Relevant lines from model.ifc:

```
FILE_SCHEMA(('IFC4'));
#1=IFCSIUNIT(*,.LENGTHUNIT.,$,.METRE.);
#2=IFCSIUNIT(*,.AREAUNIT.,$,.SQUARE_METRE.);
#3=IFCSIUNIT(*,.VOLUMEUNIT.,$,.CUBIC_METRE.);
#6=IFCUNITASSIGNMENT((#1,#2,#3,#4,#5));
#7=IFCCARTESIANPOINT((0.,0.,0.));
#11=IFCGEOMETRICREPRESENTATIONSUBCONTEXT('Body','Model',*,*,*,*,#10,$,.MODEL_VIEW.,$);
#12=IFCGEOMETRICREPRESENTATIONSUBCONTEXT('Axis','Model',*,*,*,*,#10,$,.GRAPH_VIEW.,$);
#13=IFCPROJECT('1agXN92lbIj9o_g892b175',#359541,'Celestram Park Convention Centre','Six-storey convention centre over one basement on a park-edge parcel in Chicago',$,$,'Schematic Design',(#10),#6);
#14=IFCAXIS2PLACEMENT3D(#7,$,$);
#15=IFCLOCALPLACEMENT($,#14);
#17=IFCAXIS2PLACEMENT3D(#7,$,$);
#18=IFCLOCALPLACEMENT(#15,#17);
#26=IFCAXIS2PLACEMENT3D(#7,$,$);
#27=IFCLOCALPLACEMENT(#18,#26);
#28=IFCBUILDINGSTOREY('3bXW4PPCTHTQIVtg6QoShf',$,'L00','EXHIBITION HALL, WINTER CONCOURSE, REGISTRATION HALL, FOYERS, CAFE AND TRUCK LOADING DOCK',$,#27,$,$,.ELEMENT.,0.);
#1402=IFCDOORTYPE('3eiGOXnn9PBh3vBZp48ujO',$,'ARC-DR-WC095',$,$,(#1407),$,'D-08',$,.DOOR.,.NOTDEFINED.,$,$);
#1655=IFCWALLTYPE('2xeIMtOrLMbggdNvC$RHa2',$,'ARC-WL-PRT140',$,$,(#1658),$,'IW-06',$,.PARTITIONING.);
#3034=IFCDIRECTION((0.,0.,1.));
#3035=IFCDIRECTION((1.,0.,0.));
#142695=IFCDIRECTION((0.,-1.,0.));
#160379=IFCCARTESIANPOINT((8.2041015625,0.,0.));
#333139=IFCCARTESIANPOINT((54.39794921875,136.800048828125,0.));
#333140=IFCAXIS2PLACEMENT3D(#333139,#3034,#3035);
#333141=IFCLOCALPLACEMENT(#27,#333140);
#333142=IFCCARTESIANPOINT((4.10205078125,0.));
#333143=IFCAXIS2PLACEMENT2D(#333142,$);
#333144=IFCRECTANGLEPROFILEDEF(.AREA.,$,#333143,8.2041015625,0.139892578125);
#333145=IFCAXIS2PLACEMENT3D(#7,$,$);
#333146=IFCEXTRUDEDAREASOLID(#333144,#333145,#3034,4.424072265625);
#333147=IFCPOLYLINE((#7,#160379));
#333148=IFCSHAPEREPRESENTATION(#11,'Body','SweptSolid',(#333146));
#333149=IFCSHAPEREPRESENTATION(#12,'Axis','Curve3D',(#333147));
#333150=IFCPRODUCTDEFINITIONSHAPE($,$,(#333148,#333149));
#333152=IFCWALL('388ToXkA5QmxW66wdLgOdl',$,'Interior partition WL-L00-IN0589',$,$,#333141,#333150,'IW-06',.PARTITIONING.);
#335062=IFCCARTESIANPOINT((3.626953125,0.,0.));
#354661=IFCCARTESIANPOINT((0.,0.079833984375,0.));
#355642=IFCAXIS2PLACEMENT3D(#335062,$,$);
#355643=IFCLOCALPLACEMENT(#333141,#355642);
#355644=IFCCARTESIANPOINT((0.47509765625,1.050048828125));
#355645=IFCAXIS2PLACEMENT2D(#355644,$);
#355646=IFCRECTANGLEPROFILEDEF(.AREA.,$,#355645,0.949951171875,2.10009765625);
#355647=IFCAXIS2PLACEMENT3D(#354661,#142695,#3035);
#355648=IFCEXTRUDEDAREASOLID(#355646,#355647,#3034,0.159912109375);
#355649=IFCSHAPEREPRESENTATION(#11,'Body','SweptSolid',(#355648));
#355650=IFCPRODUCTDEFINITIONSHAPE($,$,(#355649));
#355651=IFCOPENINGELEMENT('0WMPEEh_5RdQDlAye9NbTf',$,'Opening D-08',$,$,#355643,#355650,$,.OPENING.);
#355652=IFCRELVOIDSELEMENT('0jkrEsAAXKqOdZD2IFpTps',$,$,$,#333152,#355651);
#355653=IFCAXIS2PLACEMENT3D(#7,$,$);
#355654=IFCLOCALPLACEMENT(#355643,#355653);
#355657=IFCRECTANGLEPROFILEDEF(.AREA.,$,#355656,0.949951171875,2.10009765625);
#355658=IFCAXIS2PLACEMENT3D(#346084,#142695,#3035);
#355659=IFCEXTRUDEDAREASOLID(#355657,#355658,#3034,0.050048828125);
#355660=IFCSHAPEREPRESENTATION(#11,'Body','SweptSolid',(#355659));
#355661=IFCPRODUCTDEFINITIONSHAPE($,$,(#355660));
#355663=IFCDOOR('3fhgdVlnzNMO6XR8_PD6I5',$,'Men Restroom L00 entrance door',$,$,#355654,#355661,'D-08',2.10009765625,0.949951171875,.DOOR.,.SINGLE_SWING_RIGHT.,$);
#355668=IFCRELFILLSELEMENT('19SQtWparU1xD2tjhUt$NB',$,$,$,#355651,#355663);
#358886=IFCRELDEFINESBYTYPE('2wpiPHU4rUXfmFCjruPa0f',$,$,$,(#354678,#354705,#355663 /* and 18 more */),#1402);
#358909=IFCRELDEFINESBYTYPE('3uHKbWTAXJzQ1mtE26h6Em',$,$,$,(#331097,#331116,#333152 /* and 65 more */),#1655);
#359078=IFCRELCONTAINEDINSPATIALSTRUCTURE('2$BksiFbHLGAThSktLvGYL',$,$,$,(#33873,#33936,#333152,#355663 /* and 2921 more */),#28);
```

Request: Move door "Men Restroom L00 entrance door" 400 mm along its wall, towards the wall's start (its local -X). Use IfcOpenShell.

```python
import ifcopenshell
import ifcopenshell.api.geometry
import ifcopenshell.util.placement
import ifcopenshell.util.unit

model = ifcopenshell.open("model.ifc")
unit_scale = ifcopenshell.util.unit.calculate_unit_scale(model)

door = model.by_guid("3fhgdVlnzNMO6XR8_PD6I5")
opening = door.FillsVoids[0].RelatingOpeningElement
wall = opening.VoidsElements[0].RelatingBuildingElement

wall_matrix = ifcopenshell.util.placement.get_local_placement(wall.ObjectPlacement)
shift = wall_matrix[:3, 0] * -0.4 / unit_scale
before = ifcopenshell.util.placement.get_local_placement(door.ObjectPlacement)[:3, 3].copy()

# The door is placed relative to its opening, so it follows when the opening moves.
matrix = ifcopenshell.util.placement.get_local_placement(opening.ObjectPlacement)
matrix[:3, 3] += shift
ifcopenshell.api.geometry.edit_object_placement(
    model, product=opening, matrix=matrix, is_si=False, should_transform_children=True
)

after = ifcopenshell.util.placement.get_local_placement(door.ObjectPlacement)[:3, 3]
print("door moved by", (after - before).round(3) + 0.0)

model.write("model_v2.ifc")
```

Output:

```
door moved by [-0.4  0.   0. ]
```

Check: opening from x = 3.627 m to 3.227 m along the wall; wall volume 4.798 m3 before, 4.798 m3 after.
